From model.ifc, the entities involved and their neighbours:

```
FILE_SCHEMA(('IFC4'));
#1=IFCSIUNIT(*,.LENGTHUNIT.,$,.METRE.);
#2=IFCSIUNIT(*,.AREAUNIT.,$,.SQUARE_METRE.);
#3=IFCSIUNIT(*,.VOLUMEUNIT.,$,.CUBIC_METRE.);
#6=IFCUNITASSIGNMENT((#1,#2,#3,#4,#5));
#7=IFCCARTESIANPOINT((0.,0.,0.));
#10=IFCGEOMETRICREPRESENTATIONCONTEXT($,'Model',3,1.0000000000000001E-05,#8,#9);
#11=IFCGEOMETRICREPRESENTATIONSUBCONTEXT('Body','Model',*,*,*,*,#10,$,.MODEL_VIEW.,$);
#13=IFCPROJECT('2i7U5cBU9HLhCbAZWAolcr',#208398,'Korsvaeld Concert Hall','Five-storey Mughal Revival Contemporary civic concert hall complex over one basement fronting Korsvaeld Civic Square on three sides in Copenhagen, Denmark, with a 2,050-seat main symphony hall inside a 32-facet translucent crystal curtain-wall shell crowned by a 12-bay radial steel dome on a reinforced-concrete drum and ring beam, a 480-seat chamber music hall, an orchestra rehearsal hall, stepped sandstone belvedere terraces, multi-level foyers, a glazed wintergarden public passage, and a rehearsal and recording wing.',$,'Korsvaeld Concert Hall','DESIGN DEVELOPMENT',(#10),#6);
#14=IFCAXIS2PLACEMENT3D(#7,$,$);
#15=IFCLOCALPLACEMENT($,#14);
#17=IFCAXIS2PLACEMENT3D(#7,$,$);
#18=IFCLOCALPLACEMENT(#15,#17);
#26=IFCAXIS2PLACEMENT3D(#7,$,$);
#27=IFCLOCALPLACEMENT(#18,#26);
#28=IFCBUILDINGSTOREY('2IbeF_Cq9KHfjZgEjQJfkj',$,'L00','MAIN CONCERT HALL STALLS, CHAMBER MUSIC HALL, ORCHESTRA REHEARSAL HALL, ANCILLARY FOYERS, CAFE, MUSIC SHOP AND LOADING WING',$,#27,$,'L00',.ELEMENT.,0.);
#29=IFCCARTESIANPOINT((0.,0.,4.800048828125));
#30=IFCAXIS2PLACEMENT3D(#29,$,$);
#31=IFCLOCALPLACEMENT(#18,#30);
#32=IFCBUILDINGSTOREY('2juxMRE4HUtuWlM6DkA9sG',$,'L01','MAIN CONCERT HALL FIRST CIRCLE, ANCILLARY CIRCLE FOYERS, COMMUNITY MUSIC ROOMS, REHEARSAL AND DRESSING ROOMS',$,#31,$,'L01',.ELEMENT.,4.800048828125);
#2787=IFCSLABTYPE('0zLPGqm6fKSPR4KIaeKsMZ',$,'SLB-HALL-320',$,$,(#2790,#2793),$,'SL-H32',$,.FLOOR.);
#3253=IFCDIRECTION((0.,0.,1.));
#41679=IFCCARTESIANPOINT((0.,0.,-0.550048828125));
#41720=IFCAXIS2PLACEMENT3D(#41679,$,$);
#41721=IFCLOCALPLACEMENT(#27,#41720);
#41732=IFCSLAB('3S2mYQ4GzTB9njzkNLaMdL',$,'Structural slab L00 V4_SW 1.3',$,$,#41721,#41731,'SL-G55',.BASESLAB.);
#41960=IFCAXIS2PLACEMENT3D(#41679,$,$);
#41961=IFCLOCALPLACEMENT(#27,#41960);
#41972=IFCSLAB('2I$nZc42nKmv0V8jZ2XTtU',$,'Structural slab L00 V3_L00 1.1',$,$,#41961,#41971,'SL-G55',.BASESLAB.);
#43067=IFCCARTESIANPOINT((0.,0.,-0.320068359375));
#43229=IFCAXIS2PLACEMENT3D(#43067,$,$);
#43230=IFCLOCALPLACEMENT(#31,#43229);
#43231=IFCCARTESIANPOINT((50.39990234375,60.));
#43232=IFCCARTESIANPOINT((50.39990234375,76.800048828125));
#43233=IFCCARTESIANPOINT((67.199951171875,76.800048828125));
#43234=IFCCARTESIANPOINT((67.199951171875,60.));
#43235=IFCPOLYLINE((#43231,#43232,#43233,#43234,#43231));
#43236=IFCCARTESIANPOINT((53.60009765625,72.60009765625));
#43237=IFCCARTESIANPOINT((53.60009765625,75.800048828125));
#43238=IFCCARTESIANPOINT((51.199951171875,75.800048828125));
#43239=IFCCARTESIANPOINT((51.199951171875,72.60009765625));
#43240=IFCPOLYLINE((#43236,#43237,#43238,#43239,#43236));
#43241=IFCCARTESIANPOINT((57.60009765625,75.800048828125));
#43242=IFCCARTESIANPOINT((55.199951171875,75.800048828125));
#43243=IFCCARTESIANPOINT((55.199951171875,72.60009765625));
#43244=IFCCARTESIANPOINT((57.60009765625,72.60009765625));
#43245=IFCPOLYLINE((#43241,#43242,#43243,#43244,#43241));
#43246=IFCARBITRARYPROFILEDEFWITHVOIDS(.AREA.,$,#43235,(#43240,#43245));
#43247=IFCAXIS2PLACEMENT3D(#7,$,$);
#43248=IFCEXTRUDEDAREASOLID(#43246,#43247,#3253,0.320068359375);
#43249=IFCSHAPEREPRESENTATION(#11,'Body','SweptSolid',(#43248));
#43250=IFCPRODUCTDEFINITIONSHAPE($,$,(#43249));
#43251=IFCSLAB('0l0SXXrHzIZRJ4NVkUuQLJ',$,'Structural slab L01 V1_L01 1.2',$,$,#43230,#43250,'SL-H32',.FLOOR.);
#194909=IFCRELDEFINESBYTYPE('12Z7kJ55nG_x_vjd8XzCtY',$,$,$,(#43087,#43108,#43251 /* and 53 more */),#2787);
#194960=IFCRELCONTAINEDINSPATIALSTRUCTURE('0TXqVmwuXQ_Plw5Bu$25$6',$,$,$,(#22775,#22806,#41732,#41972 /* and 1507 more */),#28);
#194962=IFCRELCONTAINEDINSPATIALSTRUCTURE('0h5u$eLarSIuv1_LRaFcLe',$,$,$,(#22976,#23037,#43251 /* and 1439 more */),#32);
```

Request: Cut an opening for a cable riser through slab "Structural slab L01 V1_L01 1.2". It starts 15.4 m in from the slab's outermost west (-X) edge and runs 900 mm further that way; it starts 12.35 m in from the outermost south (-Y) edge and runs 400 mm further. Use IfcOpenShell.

```python
import numpy as np
import ifcopenshell
import ifcopenshell.api.feature
import ifcopenshell.api.geometry
import ifcopenshell.api.root
import ifcopenshell.geom
import ifcopenshell.util.placement
import ifcopenshell.util.representation
import ifcopenshell.util.shape
import ifcopenshell.util.unit

model = ifcopenshell.open("model.ifc")
unit_scale = ifcopenshell.util.unit.calculate_unit_scale(model)
settings = ifcopenshell.geom.settings()


def volume(element):
    """Net volume in cubic metres, openings subtracted."""
    shape = ifcopenshell.geom.create_shape(settings, element)
    return ifcopenshell.util.shape.get_volume(shape.geometry)


slab = model.by_guid("0l0SXXrHzIZRJ4NVkUuQLJ")
before = volume(slab)

# Extent in the slab's own axes, in metres. The edges named are its -X and -Y sides.
slab_shape = ifcopenshell.geom.create_shape(settings, slab)
vertices = ifcopenshell.util.shape.get_vertices(slab_shape.geometry)
x_min, y_min, bottom = vertices.min(axis=0)
top = vertices[:, 2].max()

opening = ifcopenshell.api.root.create_entity(model, ifc_class="IfcOpeningElement", name="Cable riser opening", predefined_type="OPENING")
context = ifcopenshell.util.representation.get_context(model, "Model", "Body", "MODEL_VIEW")
width, depth = 0.9, 0.4
outline = [(0.0, 0.0), (width, 0.0), (width, depth), (0.0, depth), (0.0, 0.0)]
# Overshoot both faces by 50 mm so the cut is clean.
shape = ifcopenshell.api.geometry.add_slab_representation(
    model, context=context, depth=top - bottom + 0.1, polyline=outline
)
ifcopenshell.api.geometry.assign_representation(model, product=opening, representation=shape)

matrix = ifcopenshell.util.placement.get_local_placement(slab.ObjectPlacement)
matrix[:, 3] = matrix @ np.append(np.array([x_min + 15.4, y_min + 12.35, bottom - 0.05]) / unit_scale, 1.0)
ifcopenshell.api.geometry.edit_object_placement(model, product=opening, matrix=matrix, is_si=False)
ifcopenshell.api.feature.add_feature(model, feature=opening, element=slab)

after = volume(slab)

print(f"slab volume {before:.3f} -> {after:.3f} m3")

model.write("model_rev.ifc")
```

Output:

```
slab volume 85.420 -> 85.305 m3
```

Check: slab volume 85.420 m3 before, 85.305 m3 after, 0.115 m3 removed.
